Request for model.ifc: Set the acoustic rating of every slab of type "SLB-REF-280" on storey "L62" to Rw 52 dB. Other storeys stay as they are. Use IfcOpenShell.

First a look at what the model holds.

```python
import ifcopenshell
import ifcopenshell.util.element

model = ifcopenshell.open("model.ifc")
print(model.schema)
storey = next(s for s in model.by_type("IfcBuildingStorey") if s.Name == "L62")
slabs = [e for e in ifcopenshell.util.element.get_decomposition(storey) if e.is_a("IfcSlab")]
seen = {}
for e in slabs:
    element_type = ifcopenshell.util.element.get_type(e)
    key = (element_type.Name if element_type != e and element_type else None, ifcopenshell.util.element.get_pset(e, "Pset_SlabCommon", "AcousticRating"))
    seen[key] = seen.get(key, 0) + 1
for (name, value), count in sorted(seen.items(), key=str):
    print(count, "x", name, "|", value)
```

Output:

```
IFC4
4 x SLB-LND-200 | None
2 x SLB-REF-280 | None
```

```python
import ifcopenshell
import ifcopenshell.api.pset
import ifcopenshell.util.element

model = ifcopenshell.open("model.ifc")

storey = next(s for s in model.by_type("IfcBuildingStorey") if s.Name == "L62")
slabs = [e for e in ifcopenshell.util.element.get_decomposition(storey) if e.is_a("IfcSlab")]

count = 0
for e in slabs:
    element_type = ifcopenshell.util.element.get_type(e)
    if element_type in (None, e) or element_type.Name != "SLB-REF-280":
        continue
    found = ifcopenshell.util.element.get_pset(e, "Pset_SlabCommon", should_inherit=False)
    if found:
        pset = model.by_id(found["id"])
        if len(ifcopenshell.util.element.get_elements_by_pset(pset)) > 1:
            pset = ifcopenshell.api.pset.unshare_pset(model, products=[e], pset=pset)[0]
    else:
        pset = ifcopenshell.api.pset.add_pset(model, product=e, name="Pset_SlabCommon")
    ifcopenshell.api.pset.edit_pset(model, pset=pset, properties={"AcousticRating": "Rw 52 dB"})
    count += 1

print(count, "slabs updated")

model.write("model_v2.ifc")
```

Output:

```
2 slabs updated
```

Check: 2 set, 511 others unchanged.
